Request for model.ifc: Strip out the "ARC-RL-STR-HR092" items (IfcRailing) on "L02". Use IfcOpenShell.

First a look at what the model holds.

```python
import ifcopenshell
import ifcopenshell.util.element

model = ifcopenshell.open("model.ifc")
print(model.schema)
storey = next(s for s in model.by_type("IfcBuildingStorey") if s.Name == "L02")
railings = [e for e in ifcopenshell.util.element.get_decomposition(storey) if e.is_a("IfcRailing")]
seen = {}
for e in railings:
    element_type = ifcopenshell.util.element.get_type(e)
    name = element_type.Name if element_type not in (None, e) else None
    seen[name] = seen.get(name, 0) + 1
for name, count in sorted(seen.items(), key=str):
    print(count, "x", name)
```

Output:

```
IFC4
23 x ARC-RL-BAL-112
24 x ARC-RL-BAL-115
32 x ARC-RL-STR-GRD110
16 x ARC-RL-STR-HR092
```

```python
import ifcopenshell
import ifcopenshell.api.root
import ifcopenshell.util.element

model = ifcopenshell.open("model.ifc")

storey = next(s for s in model.by_type("IfcBuildingStorey") if s.Name == "L02")
railings = [e for e in ifcopenshell.util.element.get_decomposition(storey) if e.is_a("IfcRailing")]
targets = [e for e in railings if (t := ifcopenshell.util.element.get_type(e)) not in (None, e) and t.Name == "ARC-RL-STR-HR092"]

for e in targets:
    ifcopenshell.api.root.remove_product(model, product=e)
print(len(targets), "removed")

model.write("model_rev.ifc")
```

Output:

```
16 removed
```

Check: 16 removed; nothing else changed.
